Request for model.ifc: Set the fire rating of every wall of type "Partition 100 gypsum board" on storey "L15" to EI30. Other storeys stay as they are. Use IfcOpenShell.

First a look at what the model holds.

```python
import ifcopenshell
import ifcopenshell.util.element

model = ifcopenshell.open("model.ifc")
print(model.schema)
storey = next(s for s in model.by_type("IfcBuildingStorey") if s.Name == "L15")
walls = [e for e in ifcopenshell.util.element.get_decomposition(storey) if e.is_a("IfcWall")]
seen = {}
for e in walls:
    element_type = ifcopenshell.util.element.get_type(e)
    key = (element_type.Name if element_type != e and element_type else None, ifcopenshell.util.element.get_pset(e, "Pset_WallCommon", "FireRating"))
    seen[key] = seen.get(key, 0) + 1
for (name, value), count in sorted(seen.items(), key=str):
    print(count, "x", name, "|", value)
```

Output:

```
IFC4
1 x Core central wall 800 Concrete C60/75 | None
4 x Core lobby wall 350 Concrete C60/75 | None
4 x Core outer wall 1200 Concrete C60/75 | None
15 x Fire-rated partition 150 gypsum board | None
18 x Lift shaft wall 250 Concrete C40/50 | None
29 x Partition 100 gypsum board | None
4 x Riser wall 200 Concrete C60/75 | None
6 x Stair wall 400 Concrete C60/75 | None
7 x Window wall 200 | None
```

```python
import ifcopenshell
import ifcopenshell.api.pset
import ifcopenshell.util.element

model = ifcopenshell.open("model.ifc")

storey = next(s for s in model.by_type("IfcBuildingStorey") if s.Name == "L15")
walls = [e for e in ifcopenshell.util.element.get_decomposition(storey) if e.is_a("IfcWall")]

count = 0
for e in walls:
    element_type = ifcopenshell.util.element.get_type(e)
    if element_type in (None, e) or element_type.Name != "Partition 100 gypsum board":
        continue
    found = ifcopenshell.util.element.get_pset(e, "Pset_WallCommon", should_inherit=False)
    if found:
        pset = model.by_id(found["id"])
        if len(ifcopenshell.util.element.get_elements_by_pset(pset)) > 1:
            pset = ifcopenshell.api.pset.unshare_pset(model, products=[e], pset=pset)[0]
    else:
        pset = ifcopenshell.api.pset.add_pset(model, product=e, name="Pset_WallCommon")
    ifcopenshell.api.pset.edit_pset(model, pset=pset, properties={"FireRating": "EI30"})
    count += 1

print(count, "walls updated")

model.write("model_updated.ifc")
```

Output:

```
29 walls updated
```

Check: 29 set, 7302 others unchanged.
